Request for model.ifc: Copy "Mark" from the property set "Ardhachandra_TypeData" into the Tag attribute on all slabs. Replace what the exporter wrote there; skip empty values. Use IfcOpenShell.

First a look at what the model holds.

```python
import ifcopenshell
import ifcopenshell.util.element

model = ifcopenshell.open("model.ifc")
print(model.schema)
slabs = model.by_type("IfcSlab")
print(len(slabs), "slabs")
for e in slabs[:8]:
    source = ifcopenshell.util.element.get_pset(e, "Ardhachandra_TypeData", "Mark")
    target = e.Tag
    print(e.id(), repr(source), repr(target), sep=" | ")
```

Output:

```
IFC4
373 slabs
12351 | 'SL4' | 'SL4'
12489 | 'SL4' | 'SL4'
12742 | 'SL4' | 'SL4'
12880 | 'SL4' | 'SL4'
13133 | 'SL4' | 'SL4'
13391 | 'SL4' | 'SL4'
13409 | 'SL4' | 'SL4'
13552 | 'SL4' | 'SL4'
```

```python
import ifcopenshell
import ifcopenshell.util.element

model = ifcopenshell.open("model.ifc")

count = 0
for e in model.by_type("IfcSlab"):
    value = ifcopenshell.util.element.get_pset(e, "Ardhachandra_TypeData", "Mark")
    current = e.Tag
    if not value or not value.strip() or current == value:
        continue
    e.Tag = value
    count += 1

print(count, "slabs updated")

model.write("model_updated.ifc")
```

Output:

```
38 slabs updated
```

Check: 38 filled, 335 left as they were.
